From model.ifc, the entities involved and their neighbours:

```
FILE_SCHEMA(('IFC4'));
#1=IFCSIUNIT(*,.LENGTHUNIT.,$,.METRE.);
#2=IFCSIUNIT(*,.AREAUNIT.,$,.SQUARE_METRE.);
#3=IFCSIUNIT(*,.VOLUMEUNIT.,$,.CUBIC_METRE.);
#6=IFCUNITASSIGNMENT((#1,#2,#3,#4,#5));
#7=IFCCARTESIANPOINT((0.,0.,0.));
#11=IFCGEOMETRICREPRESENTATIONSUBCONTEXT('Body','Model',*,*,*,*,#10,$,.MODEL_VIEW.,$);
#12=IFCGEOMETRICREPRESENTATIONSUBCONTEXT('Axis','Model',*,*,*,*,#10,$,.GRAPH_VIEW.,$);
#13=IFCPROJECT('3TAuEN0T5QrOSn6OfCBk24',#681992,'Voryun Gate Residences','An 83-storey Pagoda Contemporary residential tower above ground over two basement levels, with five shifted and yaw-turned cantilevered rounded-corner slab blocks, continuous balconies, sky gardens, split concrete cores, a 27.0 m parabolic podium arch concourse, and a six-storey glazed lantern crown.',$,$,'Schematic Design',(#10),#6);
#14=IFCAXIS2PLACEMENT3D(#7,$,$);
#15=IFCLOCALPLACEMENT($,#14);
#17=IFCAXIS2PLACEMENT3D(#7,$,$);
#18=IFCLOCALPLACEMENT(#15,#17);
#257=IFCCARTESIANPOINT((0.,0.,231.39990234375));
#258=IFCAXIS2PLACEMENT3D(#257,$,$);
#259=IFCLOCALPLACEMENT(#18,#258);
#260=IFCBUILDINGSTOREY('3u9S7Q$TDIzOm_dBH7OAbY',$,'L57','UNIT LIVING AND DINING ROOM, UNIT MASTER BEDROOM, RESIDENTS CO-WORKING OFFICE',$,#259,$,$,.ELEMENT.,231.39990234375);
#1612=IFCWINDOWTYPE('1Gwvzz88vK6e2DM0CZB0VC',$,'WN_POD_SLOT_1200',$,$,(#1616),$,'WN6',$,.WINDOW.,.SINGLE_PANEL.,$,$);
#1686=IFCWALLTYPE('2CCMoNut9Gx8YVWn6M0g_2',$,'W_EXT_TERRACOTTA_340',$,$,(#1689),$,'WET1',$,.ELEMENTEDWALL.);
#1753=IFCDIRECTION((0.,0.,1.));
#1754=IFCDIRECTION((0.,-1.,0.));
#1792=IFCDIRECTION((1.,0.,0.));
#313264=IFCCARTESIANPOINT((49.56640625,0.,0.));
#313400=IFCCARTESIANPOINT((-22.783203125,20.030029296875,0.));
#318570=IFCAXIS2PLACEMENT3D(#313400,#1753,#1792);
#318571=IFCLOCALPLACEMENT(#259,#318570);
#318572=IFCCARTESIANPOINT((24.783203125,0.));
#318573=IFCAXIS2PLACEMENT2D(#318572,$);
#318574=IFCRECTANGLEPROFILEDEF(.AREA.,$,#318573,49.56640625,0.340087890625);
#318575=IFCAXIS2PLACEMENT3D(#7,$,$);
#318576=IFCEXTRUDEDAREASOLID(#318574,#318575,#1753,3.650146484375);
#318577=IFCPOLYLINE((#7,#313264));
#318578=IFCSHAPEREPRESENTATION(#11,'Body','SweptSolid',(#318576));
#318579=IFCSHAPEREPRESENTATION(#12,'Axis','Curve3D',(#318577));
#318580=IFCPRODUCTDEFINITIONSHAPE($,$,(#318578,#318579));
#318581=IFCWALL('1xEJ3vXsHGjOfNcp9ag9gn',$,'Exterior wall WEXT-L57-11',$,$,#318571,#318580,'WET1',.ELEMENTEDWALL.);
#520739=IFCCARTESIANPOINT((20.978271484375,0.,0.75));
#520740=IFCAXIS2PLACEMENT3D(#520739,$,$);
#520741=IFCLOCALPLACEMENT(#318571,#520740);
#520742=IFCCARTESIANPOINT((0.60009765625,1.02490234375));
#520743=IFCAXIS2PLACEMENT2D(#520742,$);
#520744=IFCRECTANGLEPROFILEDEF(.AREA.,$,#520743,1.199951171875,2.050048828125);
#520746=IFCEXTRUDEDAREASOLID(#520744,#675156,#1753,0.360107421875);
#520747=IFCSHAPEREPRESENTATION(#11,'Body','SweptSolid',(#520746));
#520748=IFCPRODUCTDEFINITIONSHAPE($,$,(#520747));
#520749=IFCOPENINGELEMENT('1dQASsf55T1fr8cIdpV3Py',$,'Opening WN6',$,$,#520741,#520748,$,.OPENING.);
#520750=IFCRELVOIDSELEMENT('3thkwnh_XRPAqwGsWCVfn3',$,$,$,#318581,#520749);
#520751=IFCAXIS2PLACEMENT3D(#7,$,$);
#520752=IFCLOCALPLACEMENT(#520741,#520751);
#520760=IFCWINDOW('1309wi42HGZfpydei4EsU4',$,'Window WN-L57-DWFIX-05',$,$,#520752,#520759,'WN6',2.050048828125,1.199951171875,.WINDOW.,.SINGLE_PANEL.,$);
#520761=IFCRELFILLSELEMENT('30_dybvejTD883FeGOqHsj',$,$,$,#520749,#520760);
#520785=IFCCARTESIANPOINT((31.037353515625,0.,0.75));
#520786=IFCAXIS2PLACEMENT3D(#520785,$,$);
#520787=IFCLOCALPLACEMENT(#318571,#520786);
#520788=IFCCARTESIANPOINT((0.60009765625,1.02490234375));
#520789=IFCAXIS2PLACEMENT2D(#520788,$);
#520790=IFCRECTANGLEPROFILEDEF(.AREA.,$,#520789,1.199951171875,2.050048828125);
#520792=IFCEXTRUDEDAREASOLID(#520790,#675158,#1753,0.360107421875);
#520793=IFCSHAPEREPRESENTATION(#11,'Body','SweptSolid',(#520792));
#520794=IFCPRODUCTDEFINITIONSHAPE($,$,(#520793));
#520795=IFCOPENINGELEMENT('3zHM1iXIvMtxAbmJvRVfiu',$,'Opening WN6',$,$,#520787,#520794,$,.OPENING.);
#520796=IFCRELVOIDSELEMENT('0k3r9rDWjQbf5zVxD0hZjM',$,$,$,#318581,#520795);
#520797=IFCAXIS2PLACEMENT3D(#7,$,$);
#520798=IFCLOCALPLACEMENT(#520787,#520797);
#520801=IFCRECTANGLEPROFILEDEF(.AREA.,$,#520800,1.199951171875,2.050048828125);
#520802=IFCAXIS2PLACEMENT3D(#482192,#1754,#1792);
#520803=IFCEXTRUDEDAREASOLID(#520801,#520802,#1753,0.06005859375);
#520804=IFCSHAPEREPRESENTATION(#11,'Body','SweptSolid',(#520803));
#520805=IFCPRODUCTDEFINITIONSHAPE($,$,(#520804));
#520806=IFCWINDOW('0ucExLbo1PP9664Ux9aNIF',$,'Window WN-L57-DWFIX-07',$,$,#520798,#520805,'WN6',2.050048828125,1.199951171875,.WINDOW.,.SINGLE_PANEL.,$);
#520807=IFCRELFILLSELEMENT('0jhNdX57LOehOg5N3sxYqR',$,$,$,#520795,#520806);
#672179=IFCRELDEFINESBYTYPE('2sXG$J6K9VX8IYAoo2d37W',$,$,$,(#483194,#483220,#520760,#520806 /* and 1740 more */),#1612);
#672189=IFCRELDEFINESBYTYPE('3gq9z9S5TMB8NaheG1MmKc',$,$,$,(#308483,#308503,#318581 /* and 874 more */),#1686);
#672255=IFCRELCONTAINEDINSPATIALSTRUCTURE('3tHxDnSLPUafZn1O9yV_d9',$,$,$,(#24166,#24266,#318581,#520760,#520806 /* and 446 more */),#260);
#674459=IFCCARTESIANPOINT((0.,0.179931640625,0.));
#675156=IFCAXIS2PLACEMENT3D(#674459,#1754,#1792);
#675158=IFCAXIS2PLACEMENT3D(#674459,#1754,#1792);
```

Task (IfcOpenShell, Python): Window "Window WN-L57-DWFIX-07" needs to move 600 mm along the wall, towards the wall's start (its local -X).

```python
import ifcopenshell
import ifcopenshell.api.geometry
import ifcopenshell.util.placement

model = ifcopenshell.open("model.ifc")

window = model.by_id(520806)
opening = window.FillsVoids[0].RelatingOpeningElement
wall = opening.VoidsElements[0].RelatingBuildingElement

wall_matrix = ifcopenshell.util.placement.get_local_placement(wall.ObjectPlacement)
shift = wall_matrix[:3, 0] * -0.6
before = ifcopenshell.util.placement.get_local_placement(window.ObjectPlacement)[:3, 3].copy()

# The window is placed relative to its opening, so it follows when the opening moves.
matrix = ifcopenshell.util.placement.get_local_placement(opening.ObjectPlacement)
matrix[:3, 3] += shift
ifcopenshell.api.geometry.edit_object_placement(
    model, product=opening, matrix=matrix, is_si=False, should_transform_children=True
)

after = ifcopenshell.util.placement.get_local_placement(window.ObjectPlacement)[:3, 3]
print("window moved by", (after - before).round(3) + 0.0)

model.write("model_edited.ifc")
```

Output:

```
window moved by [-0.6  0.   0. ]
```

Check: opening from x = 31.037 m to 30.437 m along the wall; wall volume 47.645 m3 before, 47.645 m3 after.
